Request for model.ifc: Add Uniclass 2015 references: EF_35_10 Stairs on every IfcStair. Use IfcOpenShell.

First a look at what the model holds.

```python
import ifcopenshell

model = ifcopenshell.open("model.ifc")
print(model.schema)
print("classifications:", [c.Name for c in model.by_type("IfcClassification")])
for ifc_class in ("IfcDoor", "IfcRoof", "IfcStair", "IfcWall", "IfcWindow"):
    print(ifc_class, len(model.by_type(ifc_class)))
```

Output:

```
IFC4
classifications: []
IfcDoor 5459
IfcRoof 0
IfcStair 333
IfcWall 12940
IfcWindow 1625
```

```python
import ifcopenshell
import ifcopenshell.api.classification

model = ifcopenshell.open("model.ifc")

system = ifcopenshell.api.classification.add_classification(model, classification="Uniclass 2015")

codes = {
    "IfcStair": ("EF_35_10", "Stairs"),
}
for ifc_class, (code, name) in codes.items():
    products = model.by_type(ifc_class)
    ifcopenshell.api.classification.add_reference(
        model, products=products, classification=system, identification=code, name=name
    )
    print(code, len(products))

model.write("model_v2.ifc")
```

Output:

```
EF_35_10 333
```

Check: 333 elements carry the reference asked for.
